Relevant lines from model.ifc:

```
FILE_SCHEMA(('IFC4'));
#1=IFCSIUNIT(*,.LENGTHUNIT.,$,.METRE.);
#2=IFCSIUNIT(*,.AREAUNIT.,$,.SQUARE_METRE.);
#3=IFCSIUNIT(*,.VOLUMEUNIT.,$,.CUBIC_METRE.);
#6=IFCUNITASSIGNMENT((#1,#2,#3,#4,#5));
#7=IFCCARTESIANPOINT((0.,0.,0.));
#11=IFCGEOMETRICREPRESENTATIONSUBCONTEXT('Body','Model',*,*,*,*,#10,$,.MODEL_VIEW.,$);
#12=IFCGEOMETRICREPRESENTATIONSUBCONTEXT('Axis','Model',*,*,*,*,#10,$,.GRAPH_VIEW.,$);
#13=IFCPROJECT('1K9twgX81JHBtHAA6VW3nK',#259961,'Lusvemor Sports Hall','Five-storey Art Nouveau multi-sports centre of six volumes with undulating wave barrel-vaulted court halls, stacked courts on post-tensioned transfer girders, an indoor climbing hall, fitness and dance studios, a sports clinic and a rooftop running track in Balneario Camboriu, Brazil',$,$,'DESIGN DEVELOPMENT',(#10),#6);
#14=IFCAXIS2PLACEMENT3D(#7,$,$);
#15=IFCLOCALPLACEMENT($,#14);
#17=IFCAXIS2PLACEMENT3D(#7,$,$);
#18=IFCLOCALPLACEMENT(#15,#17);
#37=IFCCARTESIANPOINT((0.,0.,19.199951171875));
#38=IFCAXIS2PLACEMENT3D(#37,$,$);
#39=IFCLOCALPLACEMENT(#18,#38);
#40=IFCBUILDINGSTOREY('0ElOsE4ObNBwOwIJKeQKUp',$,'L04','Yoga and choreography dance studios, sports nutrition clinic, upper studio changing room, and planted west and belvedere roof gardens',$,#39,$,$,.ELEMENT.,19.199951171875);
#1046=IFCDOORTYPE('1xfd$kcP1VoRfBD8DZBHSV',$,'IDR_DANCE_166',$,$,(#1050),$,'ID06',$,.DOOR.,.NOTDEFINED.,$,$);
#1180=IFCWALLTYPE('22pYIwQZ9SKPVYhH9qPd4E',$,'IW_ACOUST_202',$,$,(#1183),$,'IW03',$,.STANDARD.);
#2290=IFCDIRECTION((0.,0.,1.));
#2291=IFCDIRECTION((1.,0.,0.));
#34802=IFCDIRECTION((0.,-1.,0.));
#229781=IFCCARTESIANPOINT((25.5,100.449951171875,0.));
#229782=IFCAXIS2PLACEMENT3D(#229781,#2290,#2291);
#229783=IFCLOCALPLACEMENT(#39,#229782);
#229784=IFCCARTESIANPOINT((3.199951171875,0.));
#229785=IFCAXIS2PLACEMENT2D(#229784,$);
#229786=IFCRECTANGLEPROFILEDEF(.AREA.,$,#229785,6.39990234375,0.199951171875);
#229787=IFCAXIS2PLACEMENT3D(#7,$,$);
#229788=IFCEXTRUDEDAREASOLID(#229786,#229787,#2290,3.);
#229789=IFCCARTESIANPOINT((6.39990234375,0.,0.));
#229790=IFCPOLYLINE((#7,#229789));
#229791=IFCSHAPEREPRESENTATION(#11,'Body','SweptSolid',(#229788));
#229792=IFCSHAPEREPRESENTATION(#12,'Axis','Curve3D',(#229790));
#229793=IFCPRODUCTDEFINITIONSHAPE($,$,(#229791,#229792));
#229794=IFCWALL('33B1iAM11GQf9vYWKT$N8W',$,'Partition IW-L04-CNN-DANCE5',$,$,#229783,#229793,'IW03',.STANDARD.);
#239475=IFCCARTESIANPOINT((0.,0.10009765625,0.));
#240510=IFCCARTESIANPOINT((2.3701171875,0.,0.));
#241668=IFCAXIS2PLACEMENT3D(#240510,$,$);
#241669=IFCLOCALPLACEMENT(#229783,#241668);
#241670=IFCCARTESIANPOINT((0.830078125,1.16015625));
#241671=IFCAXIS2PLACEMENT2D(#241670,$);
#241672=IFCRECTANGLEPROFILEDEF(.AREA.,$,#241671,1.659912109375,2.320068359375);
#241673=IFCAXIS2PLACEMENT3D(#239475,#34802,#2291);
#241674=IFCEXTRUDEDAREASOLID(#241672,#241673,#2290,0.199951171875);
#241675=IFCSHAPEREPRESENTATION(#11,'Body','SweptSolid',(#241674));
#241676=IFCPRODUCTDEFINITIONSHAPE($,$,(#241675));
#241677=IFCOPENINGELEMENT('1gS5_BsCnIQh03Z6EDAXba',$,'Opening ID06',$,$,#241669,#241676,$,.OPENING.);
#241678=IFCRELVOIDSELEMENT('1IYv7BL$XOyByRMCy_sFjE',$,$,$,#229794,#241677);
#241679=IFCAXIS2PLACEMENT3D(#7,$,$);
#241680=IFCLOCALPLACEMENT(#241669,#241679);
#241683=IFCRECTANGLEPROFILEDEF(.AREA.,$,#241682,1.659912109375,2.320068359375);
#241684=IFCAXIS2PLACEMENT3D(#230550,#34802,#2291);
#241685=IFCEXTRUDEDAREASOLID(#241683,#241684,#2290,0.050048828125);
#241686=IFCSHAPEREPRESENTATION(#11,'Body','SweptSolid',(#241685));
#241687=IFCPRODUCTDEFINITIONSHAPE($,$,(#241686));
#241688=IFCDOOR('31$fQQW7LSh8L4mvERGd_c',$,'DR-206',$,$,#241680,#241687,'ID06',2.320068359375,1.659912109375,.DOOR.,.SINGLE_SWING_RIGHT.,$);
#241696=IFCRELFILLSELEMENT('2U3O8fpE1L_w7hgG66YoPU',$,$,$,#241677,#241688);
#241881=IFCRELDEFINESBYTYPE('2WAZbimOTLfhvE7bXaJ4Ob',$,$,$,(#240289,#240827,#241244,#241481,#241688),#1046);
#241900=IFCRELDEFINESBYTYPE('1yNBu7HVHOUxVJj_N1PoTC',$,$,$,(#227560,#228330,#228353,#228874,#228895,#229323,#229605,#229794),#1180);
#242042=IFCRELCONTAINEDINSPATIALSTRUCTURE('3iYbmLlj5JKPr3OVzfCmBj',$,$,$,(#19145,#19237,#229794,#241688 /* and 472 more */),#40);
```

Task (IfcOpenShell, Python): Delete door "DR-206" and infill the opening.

```python
import ifcopenshell
import ifcopenshell.api.feature
import ifcopenshell.api.root
import ifcopenshell.geom
import ifcopenshell.util.shape

model = ifcopenshell.open("model.ifc")
settings = ifcopenshell.geom.settings()


def volume(element):
    """Net volume in cubic metres, openings subtracted."""
    shape = ifcopenshell.geom.create_shape(settings, element)
    return ifcopenshell.util.shape.get_volume(shape.geometry)


door = model.by_id(241688)
opening = door.FillsVoids[0].RelatingOpeningElement
wall = opening.VoidsElements[0].RelatingBuildingElement
before = volume(wall)

ifcopenshell.api.root.remove_product(model, product=door)
ifcopenshell.api.feature.remove_feature(model, feature=opening)

after = volume(wall)

print(f"wall volume {before:.3f} -> {after:.3f} m3")

model.write("model_v2.ifc")
```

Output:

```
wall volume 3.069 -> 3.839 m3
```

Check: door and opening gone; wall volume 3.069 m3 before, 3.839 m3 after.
